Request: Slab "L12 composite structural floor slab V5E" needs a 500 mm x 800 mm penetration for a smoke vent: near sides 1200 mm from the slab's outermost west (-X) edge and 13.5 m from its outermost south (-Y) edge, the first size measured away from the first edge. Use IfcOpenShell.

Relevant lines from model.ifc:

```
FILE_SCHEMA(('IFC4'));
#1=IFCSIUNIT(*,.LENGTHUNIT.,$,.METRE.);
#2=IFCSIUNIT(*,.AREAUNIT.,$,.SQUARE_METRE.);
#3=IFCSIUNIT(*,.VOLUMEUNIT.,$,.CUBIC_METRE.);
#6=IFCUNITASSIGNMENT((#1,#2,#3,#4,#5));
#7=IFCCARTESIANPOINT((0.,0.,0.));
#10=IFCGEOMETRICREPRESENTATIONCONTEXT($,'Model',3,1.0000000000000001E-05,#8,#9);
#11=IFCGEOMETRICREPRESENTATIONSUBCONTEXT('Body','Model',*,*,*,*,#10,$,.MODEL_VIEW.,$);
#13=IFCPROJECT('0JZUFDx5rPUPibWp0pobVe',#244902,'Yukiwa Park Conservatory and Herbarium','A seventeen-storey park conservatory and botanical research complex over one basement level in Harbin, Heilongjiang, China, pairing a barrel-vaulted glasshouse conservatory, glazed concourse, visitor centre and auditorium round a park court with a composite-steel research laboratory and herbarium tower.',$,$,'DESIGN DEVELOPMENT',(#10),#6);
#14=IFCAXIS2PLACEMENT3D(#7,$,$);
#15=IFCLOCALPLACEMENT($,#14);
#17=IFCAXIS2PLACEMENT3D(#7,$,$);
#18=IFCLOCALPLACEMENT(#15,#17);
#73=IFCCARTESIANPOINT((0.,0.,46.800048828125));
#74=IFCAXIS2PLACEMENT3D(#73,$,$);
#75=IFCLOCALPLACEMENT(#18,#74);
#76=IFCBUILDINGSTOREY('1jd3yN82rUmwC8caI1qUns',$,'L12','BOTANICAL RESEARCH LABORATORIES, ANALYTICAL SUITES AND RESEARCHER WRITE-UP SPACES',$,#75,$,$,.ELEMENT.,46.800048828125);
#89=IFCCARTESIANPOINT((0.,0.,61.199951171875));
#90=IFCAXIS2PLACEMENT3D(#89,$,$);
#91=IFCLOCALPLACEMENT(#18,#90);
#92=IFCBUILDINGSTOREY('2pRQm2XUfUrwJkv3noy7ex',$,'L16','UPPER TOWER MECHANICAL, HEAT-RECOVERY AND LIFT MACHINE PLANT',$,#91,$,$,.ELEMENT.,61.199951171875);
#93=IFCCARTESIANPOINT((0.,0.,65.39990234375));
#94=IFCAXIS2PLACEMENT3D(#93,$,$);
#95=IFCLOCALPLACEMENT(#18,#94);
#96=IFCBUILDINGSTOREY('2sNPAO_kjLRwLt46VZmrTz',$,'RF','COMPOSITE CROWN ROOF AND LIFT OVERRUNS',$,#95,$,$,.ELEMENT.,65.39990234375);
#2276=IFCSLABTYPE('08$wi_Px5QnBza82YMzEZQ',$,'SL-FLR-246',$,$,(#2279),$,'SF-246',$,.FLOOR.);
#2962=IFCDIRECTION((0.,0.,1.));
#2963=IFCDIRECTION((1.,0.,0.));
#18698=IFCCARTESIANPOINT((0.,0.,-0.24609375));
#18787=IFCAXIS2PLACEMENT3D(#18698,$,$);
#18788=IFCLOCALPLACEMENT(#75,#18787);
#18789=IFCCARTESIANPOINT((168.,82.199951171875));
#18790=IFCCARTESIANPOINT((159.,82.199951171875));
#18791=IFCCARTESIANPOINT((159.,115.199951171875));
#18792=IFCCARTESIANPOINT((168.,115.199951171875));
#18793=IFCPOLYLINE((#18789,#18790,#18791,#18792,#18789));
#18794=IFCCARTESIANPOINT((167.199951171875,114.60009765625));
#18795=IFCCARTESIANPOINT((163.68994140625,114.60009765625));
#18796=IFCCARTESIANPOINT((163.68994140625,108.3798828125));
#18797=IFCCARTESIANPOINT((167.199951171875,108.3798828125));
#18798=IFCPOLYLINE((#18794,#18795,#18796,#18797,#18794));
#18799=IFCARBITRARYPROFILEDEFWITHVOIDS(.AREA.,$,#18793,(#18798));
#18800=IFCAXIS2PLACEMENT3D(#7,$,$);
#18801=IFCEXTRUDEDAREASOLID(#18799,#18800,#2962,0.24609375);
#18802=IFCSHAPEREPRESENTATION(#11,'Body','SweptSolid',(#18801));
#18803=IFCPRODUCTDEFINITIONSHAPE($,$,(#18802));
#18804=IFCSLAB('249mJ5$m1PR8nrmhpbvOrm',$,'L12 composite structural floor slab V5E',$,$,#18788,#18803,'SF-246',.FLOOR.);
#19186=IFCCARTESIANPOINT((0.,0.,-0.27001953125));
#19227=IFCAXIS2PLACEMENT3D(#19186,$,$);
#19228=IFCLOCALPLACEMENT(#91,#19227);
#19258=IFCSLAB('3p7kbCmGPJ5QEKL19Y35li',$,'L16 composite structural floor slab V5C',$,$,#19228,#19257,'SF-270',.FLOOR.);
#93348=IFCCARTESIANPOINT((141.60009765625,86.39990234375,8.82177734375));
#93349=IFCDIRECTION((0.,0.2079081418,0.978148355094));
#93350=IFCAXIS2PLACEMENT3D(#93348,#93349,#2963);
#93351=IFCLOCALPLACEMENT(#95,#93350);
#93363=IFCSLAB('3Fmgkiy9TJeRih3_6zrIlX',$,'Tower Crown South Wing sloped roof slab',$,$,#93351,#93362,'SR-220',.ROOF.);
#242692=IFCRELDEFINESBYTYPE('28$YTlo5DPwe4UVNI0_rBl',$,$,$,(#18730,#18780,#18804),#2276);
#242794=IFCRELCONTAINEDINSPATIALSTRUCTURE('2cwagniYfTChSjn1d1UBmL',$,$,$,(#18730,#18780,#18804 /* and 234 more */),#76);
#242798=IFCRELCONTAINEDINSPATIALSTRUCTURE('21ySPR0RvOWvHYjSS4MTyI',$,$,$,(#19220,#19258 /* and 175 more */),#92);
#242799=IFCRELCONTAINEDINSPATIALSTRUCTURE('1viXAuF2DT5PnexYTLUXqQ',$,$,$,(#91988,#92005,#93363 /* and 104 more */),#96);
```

```python
import numpy as np
import ifcopenshell
import ifcopenshell.api.feature
import ifcopenshell.api.geometry
import ifcopenshell.api.root
import ifcopenshell.geom
import ifcopenshell.util.placement
import ifcopenshell.util.representation
import ifcopenshell.util.shape
import ifcopenshell.util.unit

model = ifcopenshell.open("model.ifc")
unit_scale = ifcopenshell.util.unit.calculate_unit_scale(model)
settings = ifcopenshell.geom.settings()


def volume(element):
    """Net volume in cubic metres, openings subtracted."""
    shape = ifcopenshell.geom.create_shape(settings, element)
    return ifcopenshell.util.shape.get_volume(shape.geometry)


slab = model.by_guid("249mJ5$m1PR8nrmhpbvOrm")
before = volume(slab)

# Extent in the slab's own axes, in metres. The edges named are its -X and -Y sides.
slab_shape = ifcopenshell.geom.create_shape(settings, slab)
vertices = ifcopenshell.util.shape.get_vertices(slab_shape.geometry)
x_min, y_min, bottom = vertices.min(axis=0)
top = vertices[:, 2].max()

opening = ifcopenshell.api.root.create_entity(model, ifc_class="IfcOpeningElement", name="Smoke vent opening", predefined_type="OPENING")
context = ifcopenshell.util.representation.get_context(model, "Model", "Body", "MODEL_VIEW")
width, depth = 0.5, 0.8
outline = [(0.0, 0.0), (width, 0.0), (width, depth), (0.0, depth), (0.0, 0.0)]
# Overshoot both faces by 50 mm so the cut is clean.
shape = ifcopenshell.api.geometry.add_slab_representation(
    model, context=context, depth=top - bottom + 0.1, polyline=outline
)
ifcopenshell.api.geometry.assign_representation(model, product=opening, representation=shape)

matrix = ifcopenshell.util.placement.get_local_placement(slab.ObjectPlacement)
matrix[:, 3] = matrix @ np.append(np.array([x_min + 1.2, y_min + 13.5, bottom - 0.05]) / unit_scale, 1.0)
ifcopenshell.api.geometry.edit_object_placement(model, product=opening, matrix=matrix, is_si=False)
ifcopenshell.api.feature.add_feature(model, feature=opening, element=slab)

after = volume(slab)

print(f"slab volume {before:.3f} -> {after:.3f} m3")

model.write("model_updated.ifc")
```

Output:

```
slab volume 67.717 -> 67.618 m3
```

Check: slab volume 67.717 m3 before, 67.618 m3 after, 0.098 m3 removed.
